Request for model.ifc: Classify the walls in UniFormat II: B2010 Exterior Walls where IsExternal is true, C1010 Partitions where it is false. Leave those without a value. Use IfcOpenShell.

First a look at what the model holds.

```python
import ifcopenshell
import ifcopenshell.util.element

model = ifcopenshell.open("model.ifc")
print(model.schema)
print("classifications:", [c.Name for c in model.by_type("IfcClassification")])
values = [ifcopenshell.util.element.get_pset(e, "Pset_WallCommon", "IsExternal") for e in model.by_type("IfcWall")]
for value in (True, False, None):
    print("IsExternal", value, values.count(value))
```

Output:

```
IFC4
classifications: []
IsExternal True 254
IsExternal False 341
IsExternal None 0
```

```python
import ifcopenshell
import ifcopenshell.api.classification
import ifcopenshell.util.element

model = ifcopenshell.open("model.ifc")

system = ifcopenshell.api.classification.add_classification(model, classification="UniFormat II")

walls = model.by_type("IfcWall")
external = {e: ifcopenshell.util.element.get_pset(e, "Pset_WallCommon", "IsExternal") for e in walls}
for flag, code, name in ((True, "B2010", "Exterior Walls"), (False, "C1010", "Partitions")):
    products = [e for e in walls if external[e] is flag]
    ifcopenshell.api.classification.add_reference(
        model, products=products, classification=system, identification=code, name=name
    )
    print(code, len(products))

model.write("model-out.ifc")
```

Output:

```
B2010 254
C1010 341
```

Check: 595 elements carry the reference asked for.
